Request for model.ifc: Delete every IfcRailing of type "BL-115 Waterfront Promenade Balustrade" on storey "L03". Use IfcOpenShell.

First a look at what the model holds.

```python
import ifcopenshell
import ifcopenshell.util.element

model = ifcopenshell.open("model.ifc")
print(model.schema)
storey = next(s for s in model.by_type("IfcBuildingStorey") if s.Name == "L03")
railings = [e for e in ifcopenshell.util.element.get_decomposition(storey) if e.is_a("IfcRailing")]
seen = {}
for e in railings:
    element_type = ifcopenshell.util.element.get_type(e)
    name = element_type.Name if element_type not in (None, e) else None
    seen[name] = seen.get(name, 0) + 1
for name, count in sorted(seen.items(), key=str):
    print(count, "x", name)
```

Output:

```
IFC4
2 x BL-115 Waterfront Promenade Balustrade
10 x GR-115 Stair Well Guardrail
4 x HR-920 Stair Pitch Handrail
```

```python
import ifcopenshell
import ifcopenshell.api.root
import ifcopenshell.util.element

model = ifcopenshell.open("model.ifc")

storey = next(s for s in model.by_type("IfcBuildingStorey") if s.Name == "L03")
railings = [e for e in ifcopenshell.util.element.get_decomposition(storey) if e.is_a("IfcRailing")]
targets = [e for e in railings if (t := ifcopenshell.util.element.get_type(e)) not in (None, e) and t.Name == "BL-115 Waterfront Promenade Balustrade"]

for e in targets:
    ifcopenshell.api.root.remove_product(model, product=e)
print(len(targets), "removed")

model.write("model_v2.ifc")
```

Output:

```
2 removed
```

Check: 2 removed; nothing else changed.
